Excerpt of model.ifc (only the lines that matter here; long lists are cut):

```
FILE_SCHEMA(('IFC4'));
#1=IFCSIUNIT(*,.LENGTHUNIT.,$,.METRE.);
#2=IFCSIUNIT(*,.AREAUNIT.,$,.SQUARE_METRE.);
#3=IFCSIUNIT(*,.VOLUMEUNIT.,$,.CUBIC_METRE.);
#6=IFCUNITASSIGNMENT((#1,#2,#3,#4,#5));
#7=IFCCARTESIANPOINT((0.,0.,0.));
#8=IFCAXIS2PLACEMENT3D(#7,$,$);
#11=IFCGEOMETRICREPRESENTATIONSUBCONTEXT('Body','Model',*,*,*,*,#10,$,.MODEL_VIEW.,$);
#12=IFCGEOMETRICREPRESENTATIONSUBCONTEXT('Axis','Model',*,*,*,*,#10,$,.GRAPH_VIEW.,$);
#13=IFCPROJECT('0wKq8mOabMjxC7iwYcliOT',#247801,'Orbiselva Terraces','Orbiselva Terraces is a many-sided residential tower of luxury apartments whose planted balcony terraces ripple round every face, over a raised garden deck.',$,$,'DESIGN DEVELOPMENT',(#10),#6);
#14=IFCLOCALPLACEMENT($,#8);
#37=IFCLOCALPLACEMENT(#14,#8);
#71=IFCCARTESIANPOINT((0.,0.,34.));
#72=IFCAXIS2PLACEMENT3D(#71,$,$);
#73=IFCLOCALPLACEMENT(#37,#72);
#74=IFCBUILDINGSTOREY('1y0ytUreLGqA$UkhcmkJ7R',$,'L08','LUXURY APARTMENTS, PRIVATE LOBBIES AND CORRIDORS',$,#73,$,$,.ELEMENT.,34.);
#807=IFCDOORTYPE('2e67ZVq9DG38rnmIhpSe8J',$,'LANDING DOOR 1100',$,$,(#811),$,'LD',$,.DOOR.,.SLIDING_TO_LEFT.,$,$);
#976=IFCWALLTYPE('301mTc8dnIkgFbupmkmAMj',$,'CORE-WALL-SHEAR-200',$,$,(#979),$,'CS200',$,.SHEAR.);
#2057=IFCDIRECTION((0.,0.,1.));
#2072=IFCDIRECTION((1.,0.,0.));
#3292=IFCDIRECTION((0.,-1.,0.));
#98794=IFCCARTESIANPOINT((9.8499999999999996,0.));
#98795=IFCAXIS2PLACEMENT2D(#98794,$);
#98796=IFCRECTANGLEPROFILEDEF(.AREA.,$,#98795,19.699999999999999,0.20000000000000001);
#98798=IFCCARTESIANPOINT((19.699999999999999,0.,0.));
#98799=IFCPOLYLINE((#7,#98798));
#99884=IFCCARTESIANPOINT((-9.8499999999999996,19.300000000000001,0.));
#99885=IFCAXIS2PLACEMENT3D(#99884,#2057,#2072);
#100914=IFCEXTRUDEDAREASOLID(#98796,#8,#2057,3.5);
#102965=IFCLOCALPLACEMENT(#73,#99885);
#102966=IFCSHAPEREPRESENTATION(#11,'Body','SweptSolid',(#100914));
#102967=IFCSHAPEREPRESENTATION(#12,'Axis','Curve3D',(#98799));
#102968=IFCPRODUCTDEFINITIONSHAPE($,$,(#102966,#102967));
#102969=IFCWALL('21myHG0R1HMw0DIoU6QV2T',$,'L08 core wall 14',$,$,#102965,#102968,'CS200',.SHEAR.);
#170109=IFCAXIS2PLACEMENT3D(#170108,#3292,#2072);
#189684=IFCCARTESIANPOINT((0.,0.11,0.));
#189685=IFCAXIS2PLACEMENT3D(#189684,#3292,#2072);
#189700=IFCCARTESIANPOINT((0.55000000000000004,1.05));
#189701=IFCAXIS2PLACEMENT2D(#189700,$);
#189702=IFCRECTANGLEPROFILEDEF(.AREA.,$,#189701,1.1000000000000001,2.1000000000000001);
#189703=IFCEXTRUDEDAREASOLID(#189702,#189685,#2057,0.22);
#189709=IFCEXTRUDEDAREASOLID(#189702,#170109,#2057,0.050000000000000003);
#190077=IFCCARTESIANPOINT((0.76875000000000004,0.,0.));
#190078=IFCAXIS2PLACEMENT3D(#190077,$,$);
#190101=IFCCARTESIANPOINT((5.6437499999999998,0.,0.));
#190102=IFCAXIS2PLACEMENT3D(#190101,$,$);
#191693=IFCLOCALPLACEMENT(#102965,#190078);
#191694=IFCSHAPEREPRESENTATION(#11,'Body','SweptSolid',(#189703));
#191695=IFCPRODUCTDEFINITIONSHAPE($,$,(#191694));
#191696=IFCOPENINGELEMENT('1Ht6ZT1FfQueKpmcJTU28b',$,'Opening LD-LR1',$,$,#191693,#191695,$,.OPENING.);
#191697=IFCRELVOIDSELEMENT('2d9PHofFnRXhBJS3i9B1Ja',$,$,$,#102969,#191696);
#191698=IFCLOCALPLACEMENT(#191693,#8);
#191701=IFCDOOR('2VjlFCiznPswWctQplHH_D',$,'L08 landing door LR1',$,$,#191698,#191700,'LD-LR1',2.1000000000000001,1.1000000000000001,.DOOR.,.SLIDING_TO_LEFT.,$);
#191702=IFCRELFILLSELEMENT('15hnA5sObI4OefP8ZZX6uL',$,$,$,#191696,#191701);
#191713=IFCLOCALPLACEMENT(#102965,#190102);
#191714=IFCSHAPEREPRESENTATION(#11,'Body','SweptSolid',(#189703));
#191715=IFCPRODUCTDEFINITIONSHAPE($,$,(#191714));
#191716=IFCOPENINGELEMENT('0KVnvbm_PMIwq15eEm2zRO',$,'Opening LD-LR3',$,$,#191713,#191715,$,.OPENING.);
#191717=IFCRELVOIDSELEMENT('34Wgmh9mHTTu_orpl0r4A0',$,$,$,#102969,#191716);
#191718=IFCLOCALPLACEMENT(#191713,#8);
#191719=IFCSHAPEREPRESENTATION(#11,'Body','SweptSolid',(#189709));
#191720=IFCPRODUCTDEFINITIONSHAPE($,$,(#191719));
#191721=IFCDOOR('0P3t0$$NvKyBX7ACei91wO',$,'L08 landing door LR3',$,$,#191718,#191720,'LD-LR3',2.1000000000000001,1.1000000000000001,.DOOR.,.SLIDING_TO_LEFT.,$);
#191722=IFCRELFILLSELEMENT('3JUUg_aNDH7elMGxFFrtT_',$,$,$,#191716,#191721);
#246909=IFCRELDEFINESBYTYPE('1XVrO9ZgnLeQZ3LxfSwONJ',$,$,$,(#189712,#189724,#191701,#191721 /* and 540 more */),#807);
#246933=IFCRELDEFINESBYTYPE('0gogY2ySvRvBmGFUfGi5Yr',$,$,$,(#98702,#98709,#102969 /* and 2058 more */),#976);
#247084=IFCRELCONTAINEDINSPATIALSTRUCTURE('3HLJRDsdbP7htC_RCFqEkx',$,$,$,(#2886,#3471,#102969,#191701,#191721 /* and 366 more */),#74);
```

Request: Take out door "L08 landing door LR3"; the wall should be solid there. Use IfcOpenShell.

```python
import ifcopenshell
import ifcopenshell.api.feature
import ifcopenshell.api.root
import ifcopenshell.geom
import ifcopenshell.util.shape

model = ifcopenshell.open("model.ifc")
settings = ifcopenshell.geom.settings()


def volume(element):
    """Net volume in cubic metres, openings subtracted."""
    shape = ifcopenshell.geom.create_shape(settings, element)
    return ifcopenshell.util.shape.get_volume(shape.geometry)


door = model.by_guid("0P3t0$$NvKyBX7ACei91wO")
opening = door.FillsVoids[0].RelatingOpeningElement
wall = opening.VoidsElements[0].RelatingBuildingElement
before = volume(wall)

ifcopenshell.api.root.remove_product(model, product=door)
ifcopenshell.api.feature.remove_feature(model, feature=opening)

after = volume(wall)

print(f"wall volume {before:.3f} -> {after:.3f} m3")

model.write("model-out.ifc")
```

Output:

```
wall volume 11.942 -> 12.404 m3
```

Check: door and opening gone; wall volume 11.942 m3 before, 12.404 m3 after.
